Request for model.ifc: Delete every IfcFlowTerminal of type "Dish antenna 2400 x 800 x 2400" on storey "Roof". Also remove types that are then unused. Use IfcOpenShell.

First a look at what the model holds.

```python
import ifcopenshell
import ifcopenshell.util.element

model = ifcopenshell.open("model.ifc")
print(model.schema)
storey = next(s for s in model.by_type("IfcBuildingStorey") if s.Name == "Roof")
terminals = [e for e in ifcopenshell.util.element.get_decomposition(storey) if e.is_a("IfcFlowTerminal")]
seen = {}
for e in terminals:
    element_type = ifcopenshell.util.element.get_type(e)
    name = element_type.Name if element_type not in (None, e) else None
    seen[name] = seen.get(name, 0) + 1
for name, count in sorted(seen.items(), key=str):
    print(count, "x", name)
```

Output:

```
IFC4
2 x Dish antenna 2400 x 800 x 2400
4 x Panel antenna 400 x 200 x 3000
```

```python
import ifcopenshell
import ifcopenshell.api.root
import ifcopenshell.util.element

model = ifcopenshell.open("model.ifc")

storey = next(s for s in model.by_type("IfcBuildingStorey") if s.Name == "Roof")
terminals = [e for e in ifcopenshell.util.element.get_decomposition(storey) if e.is_a("IfcFlowTerminal")]
targets = [e for e in terminals if (t := ifcopenshell.util.element.get_type(e)) not in (None, e) and t.Name == "Dish antenna 2400 x 800 x 2400"]
types = {ifcopenshell.util.element.get_type(e) for e in targets} - {None, *targets}

for e in targets:
    ifcopenshell.api.root.remove_product(model, product=e)
print(len(targets), "removed")

unused = [t for t in types if not ifcopenshell.util.element.get_types(t)]
for t in unused:
    ifcopenshell.api.root.remove_product(model, product=t)
print(len(unused), "unused types removed")

model.write("model-out.ifc")
```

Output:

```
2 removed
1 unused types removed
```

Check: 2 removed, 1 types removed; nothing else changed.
